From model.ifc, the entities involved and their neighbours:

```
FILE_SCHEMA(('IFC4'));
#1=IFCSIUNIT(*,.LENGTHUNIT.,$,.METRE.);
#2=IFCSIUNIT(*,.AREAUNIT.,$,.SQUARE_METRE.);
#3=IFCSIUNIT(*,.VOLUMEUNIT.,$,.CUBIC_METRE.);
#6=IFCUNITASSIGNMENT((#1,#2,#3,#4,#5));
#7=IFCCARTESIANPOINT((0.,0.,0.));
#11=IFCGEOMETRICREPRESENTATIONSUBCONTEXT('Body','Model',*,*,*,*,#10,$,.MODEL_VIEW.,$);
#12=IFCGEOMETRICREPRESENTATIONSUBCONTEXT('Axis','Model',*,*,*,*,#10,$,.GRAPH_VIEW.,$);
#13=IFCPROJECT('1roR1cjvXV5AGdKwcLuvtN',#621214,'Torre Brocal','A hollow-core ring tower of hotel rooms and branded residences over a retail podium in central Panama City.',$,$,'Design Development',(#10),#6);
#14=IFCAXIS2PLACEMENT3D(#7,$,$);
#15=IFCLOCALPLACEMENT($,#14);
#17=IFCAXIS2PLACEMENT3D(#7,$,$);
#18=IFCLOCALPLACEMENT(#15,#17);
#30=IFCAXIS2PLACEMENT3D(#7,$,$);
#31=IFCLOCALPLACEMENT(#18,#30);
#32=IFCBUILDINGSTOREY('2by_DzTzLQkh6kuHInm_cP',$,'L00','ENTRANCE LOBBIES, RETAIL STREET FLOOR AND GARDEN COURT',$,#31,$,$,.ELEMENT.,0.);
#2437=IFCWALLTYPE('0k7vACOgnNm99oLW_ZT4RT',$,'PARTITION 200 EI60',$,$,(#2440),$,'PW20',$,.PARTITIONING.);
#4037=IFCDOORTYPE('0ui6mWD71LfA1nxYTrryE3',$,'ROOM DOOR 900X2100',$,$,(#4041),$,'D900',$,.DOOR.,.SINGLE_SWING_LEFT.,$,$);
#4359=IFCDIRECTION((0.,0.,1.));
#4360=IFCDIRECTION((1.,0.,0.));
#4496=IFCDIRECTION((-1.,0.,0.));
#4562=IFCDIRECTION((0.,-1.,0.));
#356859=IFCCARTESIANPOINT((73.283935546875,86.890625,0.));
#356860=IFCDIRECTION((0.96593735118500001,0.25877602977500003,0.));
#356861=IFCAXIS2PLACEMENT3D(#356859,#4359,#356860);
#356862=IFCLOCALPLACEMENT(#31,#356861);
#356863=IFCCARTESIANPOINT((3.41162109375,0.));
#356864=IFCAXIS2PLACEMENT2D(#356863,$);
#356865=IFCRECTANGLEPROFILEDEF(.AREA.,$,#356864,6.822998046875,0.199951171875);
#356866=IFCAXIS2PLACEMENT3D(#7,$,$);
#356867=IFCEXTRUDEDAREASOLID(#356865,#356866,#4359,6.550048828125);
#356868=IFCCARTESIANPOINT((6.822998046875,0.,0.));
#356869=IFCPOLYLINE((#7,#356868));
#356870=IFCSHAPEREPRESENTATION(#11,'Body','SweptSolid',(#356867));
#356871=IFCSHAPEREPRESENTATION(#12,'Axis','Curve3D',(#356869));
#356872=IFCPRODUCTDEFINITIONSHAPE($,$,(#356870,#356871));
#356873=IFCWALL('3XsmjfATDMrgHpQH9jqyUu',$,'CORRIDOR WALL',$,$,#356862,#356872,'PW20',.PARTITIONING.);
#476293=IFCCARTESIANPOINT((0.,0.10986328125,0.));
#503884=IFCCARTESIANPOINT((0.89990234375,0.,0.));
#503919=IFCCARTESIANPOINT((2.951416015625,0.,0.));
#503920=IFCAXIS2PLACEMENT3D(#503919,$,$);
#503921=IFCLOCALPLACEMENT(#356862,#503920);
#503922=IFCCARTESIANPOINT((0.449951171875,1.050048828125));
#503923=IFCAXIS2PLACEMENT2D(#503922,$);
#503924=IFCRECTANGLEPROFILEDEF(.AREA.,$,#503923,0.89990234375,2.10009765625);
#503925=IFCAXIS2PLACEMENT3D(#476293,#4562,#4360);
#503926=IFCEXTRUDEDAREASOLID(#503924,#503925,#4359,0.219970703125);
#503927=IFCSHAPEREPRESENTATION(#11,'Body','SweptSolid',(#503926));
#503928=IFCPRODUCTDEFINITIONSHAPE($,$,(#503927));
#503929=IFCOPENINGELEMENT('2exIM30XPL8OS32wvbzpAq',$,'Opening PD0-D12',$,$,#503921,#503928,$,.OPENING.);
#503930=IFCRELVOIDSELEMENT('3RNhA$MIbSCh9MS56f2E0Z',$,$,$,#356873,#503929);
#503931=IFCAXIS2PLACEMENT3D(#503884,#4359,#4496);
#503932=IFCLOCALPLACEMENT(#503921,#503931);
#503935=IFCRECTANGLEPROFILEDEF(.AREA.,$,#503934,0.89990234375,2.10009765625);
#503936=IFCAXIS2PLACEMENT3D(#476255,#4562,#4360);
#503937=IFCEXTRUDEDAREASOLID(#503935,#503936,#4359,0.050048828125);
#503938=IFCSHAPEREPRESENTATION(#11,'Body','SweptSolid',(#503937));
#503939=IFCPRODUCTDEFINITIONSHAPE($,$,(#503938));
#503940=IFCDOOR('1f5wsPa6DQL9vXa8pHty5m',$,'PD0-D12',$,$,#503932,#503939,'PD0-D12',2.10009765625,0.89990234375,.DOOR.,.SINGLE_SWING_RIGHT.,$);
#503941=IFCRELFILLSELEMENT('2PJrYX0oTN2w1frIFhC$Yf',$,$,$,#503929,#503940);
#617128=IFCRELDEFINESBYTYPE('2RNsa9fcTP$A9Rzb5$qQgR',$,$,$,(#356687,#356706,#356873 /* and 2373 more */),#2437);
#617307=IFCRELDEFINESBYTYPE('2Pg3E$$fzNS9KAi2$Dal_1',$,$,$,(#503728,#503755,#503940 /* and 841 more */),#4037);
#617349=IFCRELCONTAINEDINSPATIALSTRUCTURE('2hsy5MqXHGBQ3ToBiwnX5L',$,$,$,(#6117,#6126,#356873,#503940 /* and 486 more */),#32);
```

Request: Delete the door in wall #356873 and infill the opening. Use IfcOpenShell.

```python
import ifcopenshell
import ifcopenshell.api.feature
import ifcopenshell.api.root
import ifcopenshell.geom
import ifcopenshell.util.shape

model = ifcopenshell.open("model.ifc")
settings = ifcopenshell.geom.settings()


def volume(element):
    """Net volume in cubic metres, openings subtracted."""
    shape = ifcopenshell.geom.create_shape(settings, element)
    return ifcopenshell.util.shape.get_volume(shape.geometry)


door = model.by_guid("1f5wsPa6DQL9vXa8pHty5m")
opening = door.FillsVoids[0].RelatingOpeningElement
wall = opening.VoidsElements[0].RelatingBuildingElement
before = volume(wall)

ifcopenshell.api.root.remove_product(model, product=door)
ifcopenshell.api.feature.remove_feature(model, feature=opening)

after = volume(wall)

print(f"wall volume {before:.3f} -> {after:.3f} m3")

model.write("model-out.ifc")
```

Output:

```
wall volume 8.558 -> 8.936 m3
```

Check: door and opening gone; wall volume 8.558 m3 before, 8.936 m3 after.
